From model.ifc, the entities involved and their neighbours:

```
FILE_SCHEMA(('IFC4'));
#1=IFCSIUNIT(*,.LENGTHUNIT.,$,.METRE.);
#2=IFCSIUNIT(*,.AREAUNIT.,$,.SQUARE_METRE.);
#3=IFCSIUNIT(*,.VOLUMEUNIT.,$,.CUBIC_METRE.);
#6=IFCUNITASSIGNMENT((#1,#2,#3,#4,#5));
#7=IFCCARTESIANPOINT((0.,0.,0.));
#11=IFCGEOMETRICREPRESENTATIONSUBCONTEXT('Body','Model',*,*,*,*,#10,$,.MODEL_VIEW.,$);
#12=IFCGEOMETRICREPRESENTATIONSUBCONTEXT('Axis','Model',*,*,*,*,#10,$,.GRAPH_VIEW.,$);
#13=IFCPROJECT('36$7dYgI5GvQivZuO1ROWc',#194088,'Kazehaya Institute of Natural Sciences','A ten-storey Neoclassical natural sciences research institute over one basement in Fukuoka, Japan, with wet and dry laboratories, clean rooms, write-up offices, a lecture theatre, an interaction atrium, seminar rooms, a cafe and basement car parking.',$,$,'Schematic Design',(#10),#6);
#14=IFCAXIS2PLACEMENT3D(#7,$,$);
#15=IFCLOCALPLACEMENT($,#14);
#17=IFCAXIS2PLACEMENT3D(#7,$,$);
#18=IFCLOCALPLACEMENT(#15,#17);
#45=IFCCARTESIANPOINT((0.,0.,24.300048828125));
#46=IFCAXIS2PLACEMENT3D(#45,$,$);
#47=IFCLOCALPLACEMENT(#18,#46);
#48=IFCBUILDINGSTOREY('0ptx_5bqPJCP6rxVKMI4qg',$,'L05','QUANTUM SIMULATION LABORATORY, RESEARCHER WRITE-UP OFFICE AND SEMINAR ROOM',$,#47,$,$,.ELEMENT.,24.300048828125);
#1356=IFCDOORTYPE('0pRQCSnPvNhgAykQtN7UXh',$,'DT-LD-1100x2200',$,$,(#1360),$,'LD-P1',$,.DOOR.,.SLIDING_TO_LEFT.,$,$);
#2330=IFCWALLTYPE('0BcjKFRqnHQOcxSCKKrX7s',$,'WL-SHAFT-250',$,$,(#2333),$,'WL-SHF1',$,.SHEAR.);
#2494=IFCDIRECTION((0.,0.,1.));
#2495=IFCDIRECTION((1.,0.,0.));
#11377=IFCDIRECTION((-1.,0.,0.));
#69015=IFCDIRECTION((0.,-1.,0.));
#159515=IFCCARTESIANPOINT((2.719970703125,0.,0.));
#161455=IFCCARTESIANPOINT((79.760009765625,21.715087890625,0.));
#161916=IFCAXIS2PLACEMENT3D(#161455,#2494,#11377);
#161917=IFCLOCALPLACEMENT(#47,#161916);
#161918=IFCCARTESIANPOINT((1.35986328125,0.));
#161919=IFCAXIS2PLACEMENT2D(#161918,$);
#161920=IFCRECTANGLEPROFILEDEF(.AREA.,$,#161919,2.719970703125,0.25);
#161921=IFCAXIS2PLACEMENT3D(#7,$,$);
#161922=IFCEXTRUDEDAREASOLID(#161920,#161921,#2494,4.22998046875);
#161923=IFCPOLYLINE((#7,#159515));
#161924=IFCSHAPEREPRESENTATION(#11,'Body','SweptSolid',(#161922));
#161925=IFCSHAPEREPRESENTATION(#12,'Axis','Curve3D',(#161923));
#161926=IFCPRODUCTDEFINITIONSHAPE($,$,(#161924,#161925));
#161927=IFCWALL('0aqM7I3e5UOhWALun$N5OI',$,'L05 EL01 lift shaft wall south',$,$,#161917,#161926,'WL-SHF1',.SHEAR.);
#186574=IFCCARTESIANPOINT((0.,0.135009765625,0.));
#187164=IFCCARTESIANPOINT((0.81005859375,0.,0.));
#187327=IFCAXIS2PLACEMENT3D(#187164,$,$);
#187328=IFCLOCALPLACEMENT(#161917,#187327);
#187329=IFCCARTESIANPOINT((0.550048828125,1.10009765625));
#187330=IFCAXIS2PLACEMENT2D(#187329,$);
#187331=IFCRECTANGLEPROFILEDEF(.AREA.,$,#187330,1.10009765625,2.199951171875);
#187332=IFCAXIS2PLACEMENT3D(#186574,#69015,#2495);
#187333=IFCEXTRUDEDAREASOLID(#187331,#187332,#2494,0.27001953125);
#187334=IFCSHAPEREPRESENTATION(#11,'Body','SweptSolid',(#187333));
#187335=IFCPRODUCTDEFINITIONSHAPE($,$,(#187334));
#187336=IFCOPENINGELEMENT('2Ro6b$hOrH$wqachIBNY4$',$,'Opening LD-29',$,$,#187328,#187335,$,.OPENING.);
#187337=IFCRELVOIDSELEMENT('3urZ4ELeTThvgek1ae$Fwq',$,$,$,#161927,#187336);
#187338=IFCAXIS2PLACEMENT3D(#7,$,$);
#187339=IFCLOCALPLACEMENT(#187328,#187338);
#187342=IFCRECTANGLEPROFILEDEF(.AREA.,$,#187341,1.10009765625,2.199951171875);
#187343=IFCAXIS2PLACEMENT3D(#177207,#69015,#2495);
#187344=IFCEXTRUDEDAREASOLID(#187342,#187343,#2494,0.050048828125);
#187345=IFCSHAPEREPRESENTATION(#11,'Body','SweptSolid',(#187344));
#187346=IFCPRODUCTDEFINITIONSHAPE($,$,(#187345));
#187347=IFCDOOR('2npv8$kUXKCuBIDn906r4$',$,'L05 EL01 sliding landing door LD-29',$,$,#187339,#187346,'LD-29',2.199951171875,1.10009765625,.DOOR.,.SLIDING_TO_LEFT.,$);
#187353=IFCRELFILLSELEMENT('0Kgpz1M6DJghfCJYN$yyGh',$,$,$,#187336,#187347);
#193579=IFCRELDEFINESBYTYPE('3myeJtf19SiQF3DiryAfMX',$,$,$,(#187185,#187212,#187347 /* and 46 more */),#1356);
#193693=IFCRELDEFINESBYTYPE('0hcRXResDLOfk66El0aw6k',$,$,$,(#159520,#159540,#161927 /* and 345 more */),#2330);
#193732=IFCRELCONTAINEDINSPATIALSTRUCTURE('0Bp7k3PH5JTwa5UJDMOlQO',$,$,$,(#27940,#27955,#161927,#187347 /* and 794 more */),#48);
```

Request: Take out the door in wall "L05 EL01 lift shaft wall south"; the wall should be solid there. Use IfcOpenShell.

```python
import ifcopenshell
import ifcopenshell.api.feature
import ifcopenshell.api.root
import ifcopenshell.geom
import ifcopenshell.util.shape

model = ifcopenshell.open("model.ifc")
settings = ifcopenshell.geom.settings()


def volume(element):
    """Net volume in cubic metres, openings subtracted."""
    shape = ifcopenshell.geom.create_shape(settings, element)
    return ifcopenshell.util.shape.get_volume(shape.geometry)


door = model.by_guid("2npv8$kUXKCuBIDn906r4$")
opening = door.FillsVoids[0].RelatingOpeningElement
wall = opening.VoidsElements[0].RelatingBuildingElement
before = volume(wall)

ifcopenshell.api.root.remove_product(model, product=door)
ifcopenshell.api.feature.remove_feature(model, feature=opening)

after = volume(wall)

print(f"wall volume {before:.3f} -> {after:.3f} m3")

model.write("model_rev.ifc")
```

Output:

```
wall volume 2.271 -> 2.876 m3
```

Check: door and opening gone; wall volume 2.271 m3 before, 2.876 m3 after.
